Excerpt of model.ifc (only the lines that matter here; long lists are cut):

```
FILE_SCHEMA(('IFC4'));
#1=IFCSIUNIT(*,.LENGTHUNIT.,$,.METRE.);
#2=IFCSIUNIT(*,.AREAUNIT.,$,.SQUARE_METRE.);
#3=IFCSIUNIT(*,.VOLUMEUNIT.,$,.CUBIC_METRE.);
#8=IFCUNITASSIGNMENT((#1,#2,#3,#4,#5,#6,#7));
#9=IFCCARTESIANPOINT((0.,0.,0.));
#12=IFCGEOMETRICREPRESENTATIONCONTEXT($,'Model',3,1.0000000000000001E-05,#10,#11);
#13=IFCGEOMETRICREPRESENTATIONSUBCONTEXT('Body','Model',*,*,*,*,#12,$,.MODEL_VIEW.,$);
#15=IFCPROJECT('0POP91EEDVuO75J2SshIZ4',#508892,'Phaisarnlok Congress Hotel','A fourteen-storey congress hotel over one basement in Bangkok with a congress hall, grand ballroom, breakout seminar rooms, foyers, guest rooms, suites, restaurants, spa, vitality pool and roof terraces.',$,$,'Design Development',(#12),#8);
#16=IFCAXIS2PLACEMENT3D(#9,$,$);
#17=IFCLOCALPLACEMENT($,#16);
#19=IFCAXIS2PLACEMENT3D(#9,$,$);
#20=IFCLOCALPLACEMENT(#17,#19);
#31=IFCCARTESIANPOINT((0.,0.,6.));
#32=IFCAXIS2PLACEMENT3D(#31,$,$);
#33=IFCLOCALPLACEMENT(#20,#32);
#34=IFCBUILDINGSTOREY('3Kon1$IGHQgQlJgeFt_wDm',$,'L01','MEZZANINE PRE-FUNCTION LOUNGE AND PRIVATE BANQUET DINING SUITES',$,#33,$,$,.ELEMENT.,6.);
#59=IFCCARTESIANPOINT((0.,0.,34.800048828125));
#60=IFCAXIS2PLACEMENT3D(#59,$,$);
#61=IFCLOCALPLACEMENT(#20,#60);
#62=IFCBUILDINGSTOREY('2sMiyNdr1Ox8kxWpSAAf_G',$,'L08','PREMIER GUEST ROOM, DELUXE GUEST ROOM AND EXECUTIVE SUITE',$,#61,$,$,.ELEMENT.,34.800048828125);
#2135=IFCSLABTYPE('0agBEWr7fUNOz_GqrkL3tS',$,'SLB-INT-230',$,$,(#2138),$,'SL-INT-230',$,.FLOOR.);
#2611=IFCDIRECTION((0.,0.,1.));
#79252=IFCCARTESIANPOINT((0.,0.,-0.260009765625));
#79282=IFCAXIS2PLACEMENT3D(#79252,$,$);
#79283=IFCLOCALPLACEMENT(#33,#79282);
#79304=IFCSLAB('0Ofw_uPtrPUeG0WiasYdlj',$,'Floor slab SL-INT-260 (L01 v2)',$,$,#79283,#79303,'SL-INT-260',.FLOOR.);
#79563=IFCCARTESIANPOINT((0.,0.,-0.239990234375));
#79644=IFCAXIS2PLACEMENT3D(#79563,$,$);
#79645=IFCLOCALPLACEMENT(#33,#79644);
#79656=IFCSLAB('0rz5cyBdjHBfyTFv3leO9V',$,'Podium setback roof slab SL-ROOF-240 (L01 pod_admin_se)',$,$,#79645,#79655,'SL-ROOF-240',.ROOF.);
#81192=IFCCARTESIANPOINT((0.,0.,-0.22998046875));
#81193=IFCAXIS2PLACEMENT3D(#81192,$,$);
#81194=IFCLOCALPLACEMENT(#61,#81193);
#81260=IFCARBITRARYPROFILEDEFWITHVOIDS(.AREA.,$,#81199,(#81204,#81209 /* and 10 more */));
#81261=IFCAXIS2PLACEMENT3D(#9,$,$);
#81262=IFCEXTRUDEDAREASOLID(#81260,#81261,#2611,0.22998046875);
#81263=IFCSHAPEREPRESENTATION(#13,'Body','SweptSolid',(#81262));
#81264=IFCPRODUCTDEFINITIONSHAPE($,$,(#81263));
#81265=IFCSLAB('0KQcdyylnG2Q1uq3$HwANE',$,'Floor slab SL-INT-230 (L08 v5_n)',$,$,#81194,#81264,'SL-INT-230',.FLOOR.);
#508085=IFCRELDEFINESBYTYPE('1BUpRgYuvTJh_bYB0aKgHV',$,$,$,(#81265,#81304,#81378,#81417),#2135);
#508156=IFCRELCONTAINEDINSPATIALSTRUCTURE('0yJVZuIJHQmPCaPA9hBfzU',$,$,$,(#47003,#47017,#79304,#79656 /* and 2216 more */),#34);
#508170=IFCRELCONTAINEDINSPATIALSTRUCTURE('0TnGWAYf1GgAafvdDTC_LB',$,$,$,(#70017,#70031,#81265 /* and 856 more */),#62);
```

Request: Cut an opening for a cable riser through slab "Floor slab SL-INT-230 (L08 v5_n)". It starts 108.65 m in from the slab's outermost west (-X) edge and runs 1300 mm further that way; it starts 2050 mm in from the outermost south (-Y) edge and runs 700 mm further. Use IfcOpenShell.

```python
import numpy as np
import ifcopenshell
import ifcopenshell.api.feature
import ifcopenshell.api.geometry
import ifcopenshell.api.root
import ifcopenshell.geom
import ifcopenshell.util.placement
import ifcopenshell.util.representation
import ifcopenshell.util.shape
import ifcopenshell.util.unit

model = ifcopenshell.open("model.ifc")
unit_scale = ifcopenshell.util.unit.calculate_unit_scale(model)
settings = ifcopenshell.geom.settings()


def volume(element):
    """Net volume in cubic metres, openings subtracted."""
    shape = ifcopenshell.geom.create_shape(settings, element)
    return ifcopenshell.util.shape.get_volume(shape.geometry)


slab = model.by_guid("0KQcdyylnG2Q1uq3$HwANE")
before = volume(slab)

# Extent in the slab's own axes, in metres. The edges named are its -X and -Y sides.
slab_shape = ifcopenshell.geom.create_shape(settings, slab)
vertices = ifcopenshell.util.shape.get_vertices(slab_shape.geometry)
x_min, y_min, bottom = vertices.min(axis=0)
top = vertices[:, 2].max()

opening = ifcopenshell.api.root.create_entity(model, ifc_class="IfcOpeningElement", name="Cable riser opening", predefined_type="OPENING")
context = ifcopenshell.util.representation.get_context(model, "Model", "Body", "MODEL_VIEW")
width, depth = 1.3, 0.7
outline = [(0.0, 0.0), (width, 0.0), (width, depth), (0.0, depth), (0.0, 0.0)]
# Overshoot both faces by 50 mm so the cut is clean.
shape = ifcopenshell.api.geometry.add_slab_representation(
    model, context=context, depth=top - bottom + 0.1, polyline=outline
)
ifcopenshell.api.geometry.assign_representation(model, product=opening, representation=shape)

matrix = ifcopenshell.util.placement.get_local_placement(slab.ObjectPlacement)
matrix[:, 3] = matrix @ np.append(np.array([x_min + 108.65, y_min + 2.05, bottom - 0.05]) / unit_scale, 1.0)
ifcopenshell.api.geometry.edit_object_placement(model, product=opening, matrix=matrix, is_si=False)
ifcopenshell.api.feature.add_feature(model, feature=opening, element=slab)

after = volume(slab)

print(f"slab volume {before:.3f} -> {after:.3f} m3")

model.write("model_edited.ifc")
```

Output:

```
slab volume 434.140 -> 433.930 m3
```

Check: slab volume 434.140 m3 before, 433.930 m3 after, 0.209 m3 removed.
